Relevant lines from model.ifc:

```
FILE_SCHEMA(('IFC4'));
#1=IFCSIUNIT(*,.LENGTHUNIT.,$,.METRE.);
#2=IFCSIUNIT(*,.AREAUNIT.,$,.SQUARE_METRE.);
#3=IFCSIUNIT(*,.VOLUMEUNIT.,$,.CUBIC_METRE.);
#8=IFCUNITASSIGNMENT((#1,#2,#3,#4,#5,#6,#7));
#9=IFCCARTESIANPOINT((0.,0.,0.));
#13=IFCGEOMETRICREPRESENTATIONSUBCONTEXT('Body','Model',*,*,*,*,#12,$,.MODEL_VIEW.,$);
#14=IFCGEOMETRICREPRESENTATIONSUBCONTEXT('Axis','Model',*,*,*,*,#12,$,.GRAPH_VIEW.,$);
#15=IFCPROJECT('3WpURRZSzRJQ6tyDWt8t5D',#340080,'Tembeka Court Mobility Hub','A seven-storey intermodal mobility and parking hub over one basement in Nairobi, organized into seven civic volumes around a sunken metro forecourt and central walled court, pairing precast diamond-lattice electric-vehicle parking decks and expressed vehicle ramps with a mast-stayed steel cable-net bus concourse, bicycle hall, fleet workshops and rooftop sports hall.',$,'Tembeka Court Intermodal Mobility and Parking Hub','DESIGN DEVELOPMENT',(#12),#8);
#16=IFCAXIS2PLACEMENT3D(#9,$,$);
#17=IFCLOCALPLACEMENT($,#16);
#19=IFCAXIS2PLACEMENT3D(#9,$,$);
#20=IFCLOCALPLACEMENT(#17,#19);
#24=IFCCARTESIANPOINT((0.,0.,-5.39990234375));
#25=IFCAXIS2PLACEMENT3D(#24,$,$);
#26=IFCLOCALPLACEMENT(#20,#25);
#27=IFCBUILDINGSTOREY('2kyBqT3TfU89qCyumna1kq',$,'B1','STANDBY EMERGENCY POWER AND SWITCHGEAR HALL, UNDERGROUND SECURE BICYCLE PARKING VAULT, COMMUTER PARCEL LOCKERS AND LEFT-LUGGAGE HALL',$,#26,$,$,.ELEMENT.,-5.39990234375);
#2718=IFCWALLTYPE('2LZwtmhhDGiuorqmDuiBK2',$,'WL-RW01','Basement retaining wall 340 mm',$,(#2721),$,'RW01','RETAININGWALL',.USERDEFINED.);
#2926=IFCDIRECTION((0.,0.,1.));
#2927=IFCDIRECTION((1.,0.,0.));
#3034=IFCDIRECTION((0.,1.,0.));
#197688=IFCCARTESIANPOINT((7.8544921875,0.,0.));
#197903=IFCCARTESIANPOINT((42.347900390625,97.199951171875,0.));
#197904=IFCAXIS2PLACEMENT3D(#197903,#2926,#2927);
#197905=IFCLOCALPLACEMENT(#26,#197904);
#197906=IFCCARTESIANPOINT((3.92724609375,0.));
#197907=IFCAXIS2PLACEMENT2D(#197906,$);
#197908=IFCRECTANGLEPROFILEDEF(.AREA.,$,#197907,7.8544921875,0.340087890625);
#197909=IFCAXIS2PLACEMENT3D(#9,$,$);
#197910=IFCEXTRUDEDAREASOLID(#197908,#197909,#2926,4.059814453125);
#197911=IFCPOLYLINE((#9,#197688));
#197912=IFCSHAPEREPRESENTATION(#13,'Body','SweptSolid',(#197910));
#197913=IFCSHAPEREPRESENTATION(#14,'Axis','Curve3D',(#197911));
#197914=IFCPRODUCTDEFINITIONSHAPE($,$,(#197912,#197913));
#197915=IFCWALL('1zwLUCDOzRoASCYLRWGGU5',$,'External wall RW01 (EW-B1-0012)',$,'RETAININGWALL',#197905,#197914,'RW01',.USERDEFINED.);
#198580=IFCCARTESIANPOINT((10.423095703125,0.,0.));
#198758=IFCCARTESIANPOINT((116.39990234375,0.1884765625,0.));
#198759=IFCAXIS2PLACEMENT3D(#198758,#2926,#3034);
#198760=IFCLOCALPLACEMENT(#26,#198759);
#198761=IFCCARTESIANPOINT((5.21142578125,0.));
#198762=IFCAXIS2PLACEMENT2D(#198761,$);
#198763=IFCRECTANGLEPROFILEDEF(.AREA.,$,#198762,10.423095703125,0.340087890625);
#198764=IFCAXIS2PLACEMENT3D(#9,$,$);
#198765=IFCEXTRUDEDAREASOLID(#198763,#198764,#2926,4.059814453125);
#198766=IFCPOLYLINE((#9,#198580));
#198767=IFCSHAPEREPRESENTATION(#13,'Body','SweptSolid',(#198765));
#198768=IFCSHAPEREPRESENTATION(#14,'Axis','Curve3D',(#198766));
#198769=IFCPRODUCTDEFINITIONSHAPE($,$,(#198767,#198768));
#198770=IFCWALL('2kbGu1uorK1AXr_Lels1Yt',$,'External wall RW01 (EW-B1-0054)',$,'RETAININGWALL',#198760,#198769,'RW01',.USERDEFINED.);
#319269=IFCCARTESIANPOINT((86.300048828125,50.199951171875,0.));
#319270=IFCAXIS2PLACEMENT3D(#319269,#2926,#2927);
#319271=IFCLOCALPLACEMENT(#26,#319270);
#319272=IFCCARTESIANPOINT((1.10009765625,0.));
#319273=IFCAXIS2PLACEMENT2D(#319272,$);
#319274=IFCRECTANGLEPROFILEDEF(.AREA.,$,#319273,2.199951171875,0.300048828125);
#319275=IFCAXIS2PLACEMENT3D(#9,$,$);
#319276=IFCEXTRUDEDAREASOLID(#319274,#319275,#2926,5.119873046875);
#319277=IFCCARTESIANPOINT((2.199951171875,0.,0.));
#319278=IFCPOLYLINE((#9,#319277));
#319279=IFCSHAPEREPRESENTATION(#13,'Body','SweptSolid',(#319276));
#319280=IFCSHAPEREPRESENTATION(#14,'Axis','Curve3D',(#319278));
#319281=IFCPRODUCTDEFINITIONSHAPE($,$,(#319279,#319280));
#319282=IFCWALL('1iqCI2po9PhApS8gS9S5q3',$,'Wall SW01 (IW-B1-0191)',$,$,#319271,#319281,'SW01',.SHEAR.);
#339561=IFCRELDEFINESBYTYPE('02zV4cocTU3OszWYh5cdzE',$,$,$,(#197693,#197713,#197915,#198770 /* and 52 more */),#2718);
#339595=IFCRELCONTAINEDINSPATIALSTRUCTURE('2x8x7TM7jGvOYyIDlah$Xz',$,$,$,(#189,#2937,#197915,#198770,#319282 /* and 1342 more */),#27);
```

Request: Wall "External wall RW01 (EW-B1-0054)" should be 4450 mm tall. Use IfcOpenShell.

```python
import ifcopenshell
import ifcopenshell.geom
import ifcopenshell.util.representation
import ifcopenshell.util.shape

model = ifcopenshell.open("model.ifc")
settings = ifcopenshell.geom.settings()


def volume(element):
    """Net volume in cubic metres, openings subtracted."""
    shape = ifcopenshell.geom.create_shape(settings, element)
    return ifcopenshell.util.shape.get_volume(shape.geometry)


wall = model.by_guid("2kbGu1uorK1AXr_Lels1Yt")
before = volume(wall)

body = ifcopenshell.util.representation.get_representation(wall, "Model", "Body")
solid = body.Items[0]
old_height = solid.Depth
solid.Depth = 4.45
after = volume(wall)

print(f"height {old_height:g} -> {solid.Depth:g}, volume {before:.3f} -> {after:.3f} m3")

model.write("model_edited.ifc")
```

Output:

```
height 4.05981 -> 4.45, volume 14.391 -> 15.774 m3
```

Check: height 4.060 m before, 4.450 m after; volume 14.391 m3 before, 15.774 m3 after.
